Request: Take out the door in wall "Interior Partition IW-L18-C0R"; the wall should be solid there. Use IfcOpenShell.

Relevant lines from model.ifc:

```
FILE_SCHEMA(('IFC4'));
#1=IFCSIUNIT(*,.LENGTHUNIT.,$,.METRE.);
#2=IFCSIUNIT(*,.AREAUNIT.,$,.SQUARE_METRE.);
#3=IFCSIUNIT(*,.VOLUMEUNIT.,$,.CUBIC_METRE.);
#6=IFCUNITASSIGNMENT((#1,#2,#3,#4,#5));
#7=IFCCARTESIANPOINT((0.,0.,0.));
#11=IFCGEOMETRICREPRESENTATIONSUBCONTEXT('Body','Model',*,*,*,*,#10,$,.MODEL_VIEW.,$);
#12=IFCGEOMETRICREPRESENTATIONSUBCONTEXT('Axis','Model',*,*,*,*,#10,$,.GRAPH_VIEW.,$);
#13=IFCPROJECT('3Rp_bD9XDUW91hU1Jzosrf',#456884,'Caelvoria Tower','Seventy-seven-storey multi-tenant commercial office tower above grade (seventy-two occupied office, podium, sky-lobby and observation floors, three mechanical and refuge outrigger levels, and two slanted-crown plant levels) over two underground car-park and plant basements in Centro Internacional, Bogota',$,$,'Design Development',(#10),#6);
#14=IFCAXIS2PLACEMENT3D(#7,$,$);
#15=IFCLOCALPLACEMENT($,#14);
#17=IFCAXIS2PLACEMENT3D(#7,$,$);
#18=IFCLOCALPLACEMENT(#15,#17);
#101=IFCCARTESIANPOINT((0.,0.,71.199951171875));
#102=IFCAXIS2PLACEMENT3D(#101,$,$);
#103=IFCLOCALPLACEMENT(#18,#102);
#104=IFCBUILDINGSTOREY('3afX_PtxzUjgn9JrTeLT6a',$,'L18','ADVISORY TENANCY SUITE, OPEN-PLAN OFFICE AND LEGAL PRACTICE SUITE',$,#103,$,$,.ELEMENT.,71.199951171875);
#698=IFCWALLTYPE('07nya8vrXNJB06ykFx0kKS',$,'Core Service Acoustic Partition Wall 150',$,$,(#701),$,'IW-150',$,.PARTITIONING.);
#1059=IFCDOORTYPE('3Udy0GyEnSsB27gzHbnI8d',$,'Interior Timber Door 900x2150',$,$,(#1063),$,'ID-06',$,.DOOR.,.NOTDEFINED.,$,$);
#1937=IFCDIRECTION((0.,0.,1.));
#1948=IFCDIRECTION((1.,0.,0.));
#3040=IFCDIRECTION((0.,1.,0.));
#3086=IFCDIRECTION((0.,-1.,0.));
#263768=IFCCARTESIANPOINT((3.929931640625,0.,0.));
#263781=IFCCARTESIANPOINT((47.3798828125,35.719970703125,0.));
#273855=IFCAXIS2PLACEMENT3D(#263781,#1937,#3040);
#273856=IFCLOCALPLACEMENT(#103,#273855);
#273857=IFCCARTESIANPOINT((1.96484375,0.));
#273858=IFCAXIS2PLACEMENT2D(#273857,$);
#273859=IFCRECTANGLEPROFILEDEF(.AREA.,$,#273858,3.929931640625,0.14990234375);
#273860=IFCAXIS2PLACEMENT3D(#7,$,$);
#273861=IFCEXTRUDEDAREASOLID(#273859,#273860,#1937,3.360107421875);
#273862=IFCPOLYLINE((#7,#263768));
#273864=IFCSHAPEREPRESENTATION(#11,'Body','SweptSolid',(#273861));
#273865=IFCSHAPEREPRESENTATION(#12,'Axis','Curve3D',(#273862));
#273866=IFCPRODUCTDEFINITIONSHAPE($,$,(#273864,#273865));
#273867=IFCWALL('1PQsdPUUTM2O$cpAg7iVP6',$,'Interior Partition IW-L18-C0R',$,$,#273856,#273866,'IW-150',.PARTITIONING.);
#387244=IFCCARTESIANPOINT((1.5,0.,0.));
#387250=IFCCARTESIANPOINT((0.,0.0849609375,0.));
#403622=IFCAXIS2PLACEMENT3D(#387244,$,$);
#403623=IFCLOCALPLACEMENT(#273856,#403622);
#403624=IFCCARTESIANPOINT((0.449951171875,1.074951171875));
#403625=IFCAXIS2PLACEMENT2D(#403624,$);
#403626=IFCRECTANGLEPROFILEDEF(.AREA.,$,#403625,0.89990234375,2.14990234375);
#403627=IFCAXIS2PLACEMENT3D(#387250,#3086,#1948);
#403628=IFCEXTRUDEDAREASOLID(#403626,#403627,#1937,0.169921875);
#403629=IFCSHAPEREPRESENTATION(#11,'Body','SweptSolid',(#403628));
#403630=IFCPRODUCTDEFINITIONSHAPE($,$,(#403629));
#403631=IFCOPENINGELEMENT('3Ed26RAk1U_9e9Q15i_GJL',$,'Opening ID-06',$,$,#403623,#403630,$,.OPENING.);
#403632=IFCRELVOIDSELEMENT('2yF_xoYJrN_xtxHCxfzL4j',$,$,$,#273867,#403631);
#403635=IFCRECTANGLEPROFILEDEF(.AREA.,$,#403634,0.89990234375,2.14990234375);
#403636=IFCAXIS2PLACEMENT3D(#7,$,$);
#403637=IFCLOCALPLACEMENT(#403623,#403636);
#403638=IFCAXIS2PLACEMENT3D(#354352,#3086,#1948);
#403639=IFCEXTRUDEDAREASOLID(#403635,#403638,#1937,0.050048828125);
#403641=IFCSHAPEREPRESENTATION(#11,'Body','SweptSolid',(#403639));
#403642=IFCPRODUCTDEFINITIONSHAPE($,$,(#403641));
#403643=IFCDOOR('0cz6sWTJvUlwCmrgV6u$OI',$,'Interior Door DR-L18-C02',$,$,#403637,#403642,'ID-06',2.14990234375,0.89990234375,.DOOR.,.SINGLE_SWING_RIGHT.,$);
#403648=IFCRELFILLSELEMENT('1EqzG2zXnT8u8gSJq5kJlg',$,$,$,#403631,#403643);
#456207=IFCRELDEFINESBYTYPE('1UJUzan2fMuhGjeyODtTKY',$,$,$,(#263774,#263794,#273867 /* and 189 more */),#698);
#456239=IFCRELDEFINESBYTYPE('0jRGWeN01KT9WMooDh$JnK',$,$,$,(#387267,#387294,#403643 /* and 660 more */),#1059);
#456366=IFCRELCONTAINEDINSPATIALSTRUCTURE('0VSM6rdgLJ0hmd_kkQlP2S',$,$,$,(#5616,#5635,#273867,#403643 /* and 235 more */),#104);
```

```python
import ifcopenshell
import ifcopenshell.api.feature
import ifcopenshell.api.root
import ifcopenshell.geom
import ifcopenshell.util.shape

model = ifcopenshell.open("model.ifc")
settings = ifcopenshell.geom.settings()


def volume(element):
    """Net volume in cubic metres, openings subtracted."""
    shape = ifcopenshell.geom.create_shape(settings, element)
    return ifcopenshell.util.shape.get_volume(shape.geometry)


door = model.by_id(403643)
opening = door.FillsVoids[0].RelatingOpeningElement
wall = opening.VoidsElements[0].RelatingBuildingElement
before = volume(wall)

ifcopenshell.api.root.remove_product(model, product=door)
ifcopenshell.api.feature.remove_feature(model, feature=opening)

after = volume(wall)

print(f"wall volume {before:.3f} -> {after:.3f} m3")

model.write("model_edited.ifc")
```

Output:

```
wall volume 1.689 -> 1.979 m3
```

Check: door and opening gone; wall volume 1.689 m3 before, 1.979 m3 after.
